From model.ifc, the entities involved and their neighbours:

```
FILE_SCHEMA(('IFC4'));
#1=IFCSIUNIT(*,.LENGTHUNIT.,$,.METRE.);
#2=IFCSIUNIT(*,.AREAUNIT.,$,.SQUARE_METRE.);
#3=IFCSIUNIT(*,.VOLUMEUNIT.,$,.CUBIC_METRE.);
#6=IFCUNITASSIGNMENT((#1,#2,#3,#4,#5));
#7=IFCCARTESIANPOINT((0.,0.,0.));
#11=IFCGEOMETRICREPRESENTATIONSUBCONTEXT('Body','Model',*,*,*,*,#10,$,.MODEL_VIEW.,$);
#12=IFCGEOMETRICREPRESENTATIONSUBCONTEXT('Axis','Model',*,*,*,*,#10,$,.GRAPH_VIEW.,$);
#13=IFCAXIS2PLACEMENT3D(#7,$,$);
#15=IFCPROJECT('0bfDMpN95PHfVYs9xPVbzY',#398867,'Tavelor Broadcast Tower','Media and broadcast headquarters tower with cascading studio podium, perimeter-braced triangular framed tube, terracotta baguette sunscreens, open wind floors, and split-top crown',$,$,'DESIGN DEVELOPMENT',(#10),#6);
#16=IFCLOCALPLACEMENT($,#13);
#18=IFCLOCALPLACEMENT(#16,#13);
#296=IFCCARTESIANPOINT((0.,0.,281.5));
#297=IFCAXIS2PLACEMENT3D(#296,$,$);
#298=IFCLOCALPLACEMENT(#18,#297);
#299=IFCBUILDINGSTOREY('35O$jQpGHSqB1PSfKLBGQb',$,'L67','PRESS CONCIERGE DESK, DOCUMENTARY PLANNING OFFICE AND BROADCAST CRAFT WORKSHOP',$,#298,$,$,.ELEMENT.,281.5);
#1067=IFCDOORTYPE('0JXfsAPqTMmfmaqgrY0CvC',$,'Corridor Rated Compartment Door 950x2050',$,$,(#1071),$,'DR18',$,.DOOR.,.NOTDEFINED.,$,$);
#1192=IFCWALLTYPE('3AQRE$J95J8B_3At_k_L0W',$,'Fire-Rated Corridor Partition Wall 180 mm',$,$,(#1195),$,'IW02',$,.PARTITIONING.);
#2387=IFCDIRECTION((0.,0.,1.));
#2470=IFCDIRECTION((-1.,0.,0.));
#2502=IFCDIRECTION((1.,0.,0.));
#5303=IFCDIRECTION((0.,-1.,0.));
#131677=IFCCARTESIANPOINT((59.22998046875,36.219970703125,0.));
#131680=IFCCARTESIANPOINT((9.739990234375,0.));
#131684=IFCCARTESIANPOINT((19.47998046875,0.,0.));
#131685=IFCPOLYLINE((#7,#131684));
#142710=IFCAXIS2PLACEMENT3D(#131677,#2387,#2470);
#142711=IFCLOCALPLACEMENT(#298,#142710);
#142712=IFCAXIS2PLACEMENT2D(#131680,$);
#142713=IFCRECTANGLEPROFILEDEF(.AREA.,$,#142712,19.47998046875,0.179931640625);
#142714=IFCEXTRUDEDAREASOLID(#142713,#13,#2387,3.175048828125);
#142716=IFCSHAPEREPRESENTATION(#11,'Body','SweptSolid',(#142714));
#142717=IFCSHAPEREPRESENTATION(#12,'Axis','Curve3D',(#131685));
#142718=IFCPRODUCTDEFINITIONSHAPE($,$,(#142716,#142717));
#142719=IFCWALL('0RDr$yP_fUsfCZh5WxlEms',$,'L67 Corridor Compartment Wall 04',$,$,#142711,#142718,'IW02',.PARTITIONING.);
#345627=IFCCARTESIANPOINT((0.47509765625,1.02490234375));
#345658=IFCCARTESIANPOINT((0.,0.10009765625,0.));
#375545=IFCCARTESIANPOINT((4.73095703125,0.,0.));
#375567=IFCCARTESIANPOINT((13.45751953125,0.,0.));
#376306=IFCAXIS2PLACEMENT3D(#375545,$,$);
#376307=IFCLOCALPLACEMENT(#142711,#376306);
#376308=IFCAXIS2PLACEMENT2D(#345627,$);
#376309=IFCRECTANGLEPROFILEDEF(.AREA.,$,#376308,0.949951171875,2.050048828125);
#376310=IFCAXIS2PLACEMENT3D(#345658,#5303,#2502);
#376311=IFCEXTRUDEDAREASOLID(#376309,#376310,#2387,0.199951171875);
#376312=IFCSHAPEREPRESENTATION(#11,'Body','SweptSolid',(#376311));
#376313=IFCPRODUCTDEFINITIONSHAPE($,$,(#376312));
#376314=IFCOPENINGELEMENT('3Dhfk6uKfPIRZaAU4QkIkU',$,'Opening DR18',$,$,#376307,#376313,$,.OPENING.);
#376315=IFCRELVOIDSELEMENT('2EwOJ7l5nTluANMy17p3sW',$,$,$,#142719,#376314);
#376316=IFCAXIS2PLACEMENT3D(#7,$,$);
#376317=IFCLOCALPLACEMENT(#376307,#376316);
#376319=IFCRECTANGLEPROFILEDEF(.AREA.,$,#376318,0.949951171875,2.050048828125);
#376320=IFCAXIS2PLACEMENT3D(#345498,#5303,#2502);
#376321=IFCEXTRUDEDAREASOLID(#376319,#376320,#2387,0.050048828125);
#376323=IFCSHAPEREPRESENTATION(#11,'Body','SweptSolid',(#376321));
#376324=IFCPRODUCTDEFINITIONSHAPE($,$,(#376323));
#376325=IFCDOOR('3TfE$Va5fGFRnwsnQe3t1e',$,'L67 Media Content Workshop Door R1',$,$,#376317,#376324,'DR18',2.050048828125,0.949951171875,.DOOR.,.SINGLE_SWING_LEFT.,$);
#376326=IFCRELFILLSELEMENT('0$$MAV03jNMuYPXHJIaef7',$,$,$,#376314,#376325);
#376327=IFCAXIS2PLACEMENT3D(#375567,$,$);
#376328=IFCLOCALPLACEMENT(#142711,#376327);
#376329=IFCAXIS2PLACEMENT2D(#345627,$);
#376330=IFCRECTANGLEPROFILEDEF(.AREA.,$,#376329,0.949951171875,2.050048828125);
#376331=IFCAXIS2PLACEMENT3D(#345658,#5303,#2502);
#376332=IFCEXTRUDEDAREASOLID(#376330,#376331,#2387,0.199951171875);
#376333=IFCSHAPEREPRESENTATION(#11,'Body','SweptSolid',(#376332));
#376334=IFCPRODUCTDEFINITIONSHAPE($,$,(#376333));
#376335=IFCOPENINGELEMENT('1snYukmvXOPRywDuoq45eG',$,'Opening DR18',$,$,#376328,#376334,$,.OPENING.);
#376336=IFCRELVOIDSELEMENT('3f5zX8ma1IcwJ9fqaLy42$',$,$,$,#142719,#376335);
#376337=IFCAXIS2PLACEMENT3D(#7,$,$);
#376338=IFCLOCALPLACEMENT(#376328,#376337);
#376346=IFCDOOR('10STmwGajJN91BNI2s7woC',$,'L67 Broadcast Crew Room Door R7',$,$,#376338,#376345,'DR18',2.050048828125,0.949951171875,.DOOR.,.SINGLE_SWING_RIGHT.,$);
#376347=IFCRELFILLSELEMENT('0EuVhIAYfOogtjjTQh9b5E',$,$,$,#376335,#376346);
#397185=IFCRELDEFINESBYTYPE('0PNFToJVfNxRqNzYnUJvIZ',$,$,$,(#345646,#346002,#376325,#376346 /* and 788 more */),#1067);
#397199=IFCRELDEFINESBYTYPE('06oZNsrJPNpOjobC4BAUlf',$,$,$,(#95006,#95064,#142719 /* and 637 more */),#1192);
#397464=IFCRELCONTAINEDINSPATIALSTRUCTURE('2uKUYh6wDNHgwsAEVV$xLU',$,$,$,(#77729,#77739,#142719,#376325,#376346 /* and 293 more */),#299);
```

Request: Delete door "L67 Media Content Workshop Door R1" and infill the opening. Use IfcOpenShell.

```python
import ifcopenshell
import ifcopenshell.api.feature
import ifcopenshell.api.root
import ifcopenshell.geom
import ifcopenshell.util.shape

model = ifcopenshell.open("model.ifc")
settings = ifcopenshell.geom.settings()


def volume(element):
    """Net volume in cubic metres, openings subtracted."""
    shape = ifcopenshell.geom.create_shape(settings, element)
    return ifcopenshell.util.shape.get_volume(shape.geometry)


door = model.by_guid("3TfE$Va5fGFRnwsnQe3t1e")
opening = door.FillsVoids[0].RelatingOpeningElement
wall = opening.VoidsElements[0].RelatingBuildingElement
before = volume(wall)

ifcopenshell.api.root.remove_product(model, product=door)
ifcopenshell.api.feature.remove_feature(model, feature=opening)

after = volume(wall)

print(f"wall volume {before:.3f} -> {after:.3f} m3")

model.write("model-out.ifc")
```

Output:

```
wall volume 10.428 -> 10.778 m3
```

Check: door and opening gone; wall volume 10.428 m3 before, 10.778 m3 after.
